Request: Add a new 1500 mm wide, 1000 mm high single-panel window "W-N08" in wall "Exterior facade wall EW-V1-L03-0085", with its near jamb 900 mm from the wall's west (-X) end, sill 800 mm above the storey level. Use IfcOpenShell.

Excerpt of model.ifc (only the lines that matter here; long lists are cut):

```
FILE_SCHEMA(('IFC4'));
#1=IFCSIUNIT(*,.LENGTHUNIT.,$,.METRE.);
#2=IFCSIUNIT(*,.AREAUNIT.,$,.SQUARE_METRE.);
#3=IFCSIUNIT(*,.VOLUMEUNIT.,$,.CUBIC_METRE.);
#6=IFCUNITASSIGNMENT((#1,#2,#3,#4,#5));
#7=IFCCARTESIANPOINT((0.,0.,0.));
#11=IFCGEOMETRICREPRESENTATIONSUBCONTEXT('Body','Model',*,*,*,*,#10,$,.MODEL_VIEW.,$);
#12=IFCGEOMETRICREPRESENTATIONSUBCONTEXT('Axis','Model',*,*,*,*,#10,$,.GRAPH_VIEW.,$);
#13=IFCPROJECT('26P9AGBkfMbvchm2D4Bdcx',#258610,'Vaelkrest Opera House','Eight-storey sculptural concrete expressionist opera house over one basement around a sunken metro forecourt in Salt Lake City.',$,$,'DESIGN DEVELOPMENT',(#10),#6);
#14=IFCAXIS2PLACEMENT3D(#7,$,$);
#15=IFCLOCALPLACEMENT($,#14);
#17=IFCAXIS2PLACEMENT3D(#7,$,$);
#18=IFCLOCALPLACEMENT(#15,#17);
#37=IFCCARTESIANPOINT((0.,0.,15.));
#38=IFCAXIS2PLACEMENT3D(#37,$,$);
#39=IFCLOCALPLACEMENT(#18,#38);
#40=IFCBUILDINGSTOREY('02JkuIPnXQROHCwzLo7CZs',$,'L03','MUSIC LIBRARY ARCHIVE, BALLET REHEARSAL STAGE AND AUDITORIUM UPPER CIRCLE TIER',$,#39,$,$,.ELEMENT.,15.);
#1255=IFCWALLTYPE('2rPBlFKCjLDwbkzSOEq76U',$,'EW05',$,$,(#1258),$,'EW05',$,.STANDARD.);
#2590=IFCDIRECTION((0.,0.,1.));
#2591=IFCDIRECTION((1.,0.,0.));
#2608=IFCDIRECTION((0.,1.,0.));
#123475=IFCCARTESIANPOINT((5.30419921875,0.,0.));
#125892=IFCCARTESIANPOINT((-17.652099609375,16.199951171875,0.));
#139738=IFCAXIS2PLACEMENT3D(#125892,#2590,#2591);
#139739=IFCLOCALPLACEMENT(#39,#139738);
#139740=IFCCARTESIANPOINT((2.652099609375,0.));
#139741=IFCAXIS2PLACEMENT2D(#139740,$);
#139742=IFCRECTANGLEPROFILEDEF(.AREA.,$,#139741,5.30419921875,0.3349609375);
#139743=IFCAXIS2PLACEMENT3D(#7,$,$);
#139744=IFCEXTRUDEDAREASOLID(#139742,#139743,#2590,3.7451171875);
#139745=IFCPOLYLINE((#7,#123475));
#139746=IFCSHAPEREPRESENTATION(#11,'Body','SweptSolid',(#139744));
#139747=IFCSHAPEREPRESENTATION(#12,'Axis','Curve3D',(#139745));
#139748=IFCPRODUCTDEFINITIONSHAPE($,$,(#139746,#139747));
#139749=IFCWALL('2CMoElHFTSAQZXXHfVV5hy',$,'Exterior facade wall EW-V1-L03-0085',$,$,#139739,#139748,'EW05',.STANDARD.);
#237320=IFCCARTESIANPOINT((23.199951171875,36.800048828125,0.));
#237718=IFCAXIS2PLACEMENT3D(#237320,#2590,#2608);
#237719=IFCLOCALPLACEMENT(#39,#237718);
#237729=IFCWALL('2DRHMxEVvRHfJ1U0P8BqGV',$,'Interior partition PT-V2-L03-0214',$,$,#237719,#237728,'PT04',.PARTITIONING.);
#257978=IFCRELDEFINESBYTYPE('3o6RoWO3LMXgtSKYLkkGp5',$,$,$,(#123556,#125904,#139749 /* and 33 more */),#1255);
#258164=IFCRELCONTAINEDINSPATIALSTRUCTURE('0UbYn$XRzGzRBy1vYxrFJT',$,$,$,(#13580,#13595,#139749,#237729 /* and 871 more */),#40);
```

```python
import numpy as np
import ifcopenshell
import ifcopenshell.api.feature
import ifcopenshell.api.geometry
import ifcopenshell.api.root
import ifcopenshell.api.spatial
import ifcopenshell.geom
import ifcopenshell.util.element
import ifcopenshell.util.placement
import ifcopenshell.util.representation
import ifcopenshell.util.shape
import ifcopenshell.util.unit

model = ifcopenshell.open("model.ifc")
unit_scale = ifcopenshell.util.unit.calculate_unit_scale(model)
settings = ifcopenshell.geom.settings()


def volume(element):
    """Net volume in cubic metres, openings subtracted."""
    shape = ifcopenshell.geom.create_shape(settings, element)
    return ifcopenshell.util.shape.get_volume(shape.geometry)


wall = model.by_guid("2CMoElHFTSAQZXXHfVV5hy")
storey = ifcopenshell.util.element.get_container(wall, ifc_class="IfcBuildingStorey")
context = ifcopenshell.util.representation.get_context(model, "Model", "Body", "MODEL_VIEW")
before = volume(wall)

width, height, from_end, sill = 1.5, 1, 0.9, 0.8  # metres

# The wall runs along its own X axis, and the end named is its -X end.
wall_shape = ifcopenshell.geom.create_shape(settings, wall)
x, y, z = ifcopenshell.util.shape.get_vertices(wall_shape.geometry).T
start = x.min() + from_end
face, thickness = float(y.min()), float(y.max() - y.min())
wall_matrix = ifcopenshell.util.placement.get_local_placement(wall.ObjectPlacement)
level = ifcopenshell.util.placement.get_local_placement(storey.ObjectPlacement)[2, 3]


def in_wall(x, y):
    """Placement at x, y metres in the wall's axes, at sill height."""
    matrix = wall_matrix.copy()
    matrix[:, 3] = wall_matrix @ np.array([x / unit_scale, y / unit_scale, 0.0, 1.0])
    matrix[2, 3] = level + sill / unit_scale
    return matrix


# Opening: a box that overshoots both wall faces by 50 mm.
opening = ifcopenshell.api.root.create_entity(model, ifc_class="IfcOpeningElement", predefined_type="OPENING")
box = ifcopenshell.api.geometry.add_wall_representation(
    model, context=context, length=width, height=height, thickness=thickness + 0.1
)
ifcopenshell.api.geometry.assign_representation(model, product=opening, representation=box)
ifcopenshell.api.geometry.edit_object_placement(model, product=opening, matrix=in_wall(start, face - 0.05), is_si=False)
ifcopenshell.api.feature.add_feature(model, feature=opening, element=wall)

window = ifcopenshell.api.root.create_entity(model, ifc_class="IfcWindow", name="W-N08", predefined_type="WINDOW")
window.OverallWidth, window.OverallHeight = width / unit_scale, height / unit_scale
window.PartitioningType = "SINGLE_PANEL"
body = ifcopenshell.api.geometry.add_window_representation(
    model,
    context=context,
    overall_width=window.OverallWidth,
    overall_height=window.OverallHeight,
    partition_type="SINGLE_PANEL",
)
ifcopenshell.api.geometry.assign_representation(model, product=window, representation=body)
ifcopenshell.api.spatial.assign_container(model, products=[window], relating_structure=storey)
ifcopenshell.api.feature.add_filling(model, opening=opening, element=window)

# Centre the window in the wall's thickness.
ifcopenshell.api.geometry.edit_object_placement(model, product=window, matrix=in_wall(start, face), is_si=False)
window_shape = ifcopenshell.geom.create_shape(settings, window)
depth = ifcopenshell.util.shape.get_vertices(window_shape.geometry)[:, 1]
offset = face + thickness / 2 - (depth.min() + depth.max()) / 2
ifcopenshell.api.geometry.edit_object_placement(model, product=window, matrix=in_wall(start, offset), is_si=False)

after = volume(wall)

print(f"wall volume {before:.3f} -> {after:.3f} m3")

model.write("model_rev.ifc")
```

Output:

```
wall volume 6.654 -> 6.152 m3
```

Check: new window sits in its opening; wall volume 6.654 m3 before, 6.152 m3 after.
